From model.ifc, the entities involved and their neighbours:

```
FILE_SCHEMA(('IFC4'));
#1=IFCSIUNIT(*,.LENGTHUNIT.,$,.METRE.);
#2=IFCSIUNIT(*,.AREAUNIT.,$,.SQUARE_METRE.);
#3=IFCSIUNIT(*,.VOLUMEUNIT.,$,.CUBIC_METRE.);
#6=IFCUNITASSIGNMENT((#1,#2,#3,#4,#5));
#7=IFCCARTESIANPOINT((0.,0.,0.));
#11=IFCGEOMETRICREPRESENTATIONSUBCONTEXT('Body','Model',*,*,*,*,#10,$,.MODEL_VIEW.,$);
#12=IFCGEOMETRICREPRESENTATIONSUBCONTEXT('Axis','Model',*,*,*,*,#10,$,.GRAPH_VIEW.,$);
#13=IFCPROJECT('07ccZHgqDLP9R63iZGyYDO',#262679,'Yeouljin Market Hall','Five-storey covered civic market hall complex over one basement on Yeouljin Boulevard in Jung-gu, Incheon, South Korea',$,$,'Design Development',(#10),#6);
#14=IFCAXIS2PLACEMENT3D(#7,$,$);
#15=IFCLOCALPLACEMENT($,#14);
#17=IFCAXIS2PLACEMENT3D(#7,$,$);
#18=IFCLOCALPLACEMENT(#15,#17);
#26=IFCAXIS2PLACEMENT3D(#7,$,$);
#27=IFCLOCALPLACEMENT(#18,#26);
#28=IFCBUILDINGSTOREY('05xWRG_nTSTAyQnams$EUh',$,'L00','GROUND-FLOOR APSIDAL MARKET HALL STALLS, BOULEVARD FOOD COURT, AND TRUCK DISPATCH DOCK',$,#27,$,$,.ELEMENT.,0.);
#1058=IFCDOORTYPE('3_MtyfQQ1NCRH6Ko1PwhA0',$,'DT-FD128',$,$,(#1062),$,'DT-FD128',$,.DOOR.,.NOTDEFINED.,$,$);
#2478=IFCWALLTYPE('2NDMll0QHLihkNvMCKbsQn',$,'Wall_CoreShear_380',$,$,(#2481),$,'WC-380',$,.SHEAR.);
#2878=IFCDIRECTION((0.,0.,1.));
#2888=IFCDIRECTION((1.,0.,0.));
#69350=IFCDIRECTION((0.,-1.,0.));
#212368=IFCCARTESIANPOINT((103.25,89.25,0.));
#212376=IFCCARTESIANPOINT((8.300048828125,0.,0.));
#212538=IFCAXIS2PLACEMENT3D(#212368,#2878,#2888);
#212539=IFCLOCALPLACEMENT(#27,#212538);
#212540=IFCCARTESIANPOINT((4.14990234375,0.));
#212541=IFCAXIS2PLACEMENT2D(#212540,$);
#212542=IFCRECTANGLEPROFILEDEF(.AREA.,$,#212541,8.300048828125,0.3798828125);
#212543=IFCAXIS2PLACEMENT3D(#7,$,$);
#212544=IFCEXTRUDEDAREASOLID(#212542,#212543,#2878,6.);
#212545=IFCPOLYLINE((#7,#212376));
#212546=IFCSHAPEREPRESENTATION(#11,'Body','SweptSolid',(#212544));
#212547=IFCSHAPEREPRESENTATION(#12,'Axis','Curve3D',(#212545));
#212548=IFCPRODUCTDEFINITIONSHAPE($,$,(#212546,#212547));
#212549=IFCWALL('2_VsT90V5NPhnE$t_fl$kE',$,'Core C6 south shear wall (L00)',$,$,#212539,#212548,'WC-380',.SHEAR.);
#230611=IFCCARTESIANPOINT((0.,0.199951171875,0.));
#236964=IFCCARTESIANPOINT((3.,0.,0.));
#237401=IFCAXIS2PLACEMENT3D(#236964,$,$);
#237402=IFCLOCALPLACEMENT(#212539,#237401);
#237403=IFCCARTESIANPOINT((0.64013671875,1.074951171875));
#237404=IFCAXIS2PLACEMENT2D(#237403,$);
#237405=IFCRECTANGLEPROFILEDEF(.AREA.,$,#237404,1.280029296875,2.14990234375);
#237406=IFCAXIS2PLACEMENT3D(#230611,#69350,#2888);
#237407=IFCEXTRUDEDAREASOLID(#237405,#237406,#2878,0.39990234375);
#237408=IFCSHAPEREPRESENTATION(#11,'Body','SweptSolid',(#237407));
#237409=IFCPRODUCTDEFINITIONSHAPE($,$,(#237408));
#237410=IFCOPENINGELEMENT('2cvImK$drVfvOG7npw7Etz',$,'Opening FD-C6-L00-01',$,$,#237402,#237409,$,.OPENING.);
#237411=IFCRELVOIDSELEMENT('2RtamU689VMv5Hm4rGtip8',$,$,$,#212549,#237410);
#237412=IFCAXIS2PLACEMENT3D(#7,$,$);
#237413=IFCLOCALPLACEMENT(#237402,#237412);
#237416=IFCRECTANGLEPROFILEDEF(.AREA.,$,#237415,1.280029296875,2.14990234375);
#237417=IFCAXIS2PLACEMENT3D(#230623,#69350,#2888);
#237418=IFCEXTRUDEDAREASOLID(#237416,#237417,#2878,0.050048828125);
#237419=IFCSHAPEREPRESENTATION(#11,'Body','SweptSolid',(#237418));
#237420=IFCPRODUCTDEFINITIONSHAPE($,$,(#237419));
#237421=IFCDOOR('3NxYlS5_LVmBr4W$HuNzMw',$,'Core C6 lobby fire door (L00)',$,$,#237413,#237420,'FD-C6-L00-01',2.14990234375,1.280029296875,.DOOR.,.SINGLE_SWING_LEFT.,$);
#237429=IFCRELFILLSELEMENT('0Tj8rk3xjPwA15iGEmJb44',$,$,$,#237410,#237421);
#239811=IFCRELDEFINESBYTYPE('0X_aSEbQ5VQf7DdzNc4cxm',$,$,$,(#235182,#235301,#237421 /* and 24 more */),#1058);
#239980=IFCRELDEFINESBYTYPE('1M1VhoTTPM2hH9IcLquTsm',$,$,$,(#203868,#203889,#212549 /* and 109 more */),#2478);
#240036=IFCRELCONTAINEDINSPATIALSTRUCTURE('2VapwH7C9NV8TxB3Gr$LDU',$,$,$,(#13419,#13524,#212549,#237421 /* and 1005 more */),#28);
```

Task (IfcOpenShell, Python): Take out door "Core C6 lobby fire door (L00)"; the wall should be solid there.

```python
import ifcopenshell
import ifcopenshell.api.feature
import ifcopenshell.api.root
import ifcopenshell.geom
import ifcopenshell.util.shape

model = ifcopenshell.open("model.ifc")
settings = ifcopenshell.geom.settings()


def volume(element):
    """Net volume in cubic metres, openings subtracted."""
    shape = ifcopenshell.geom.create_shape(settings, element)
    return ifcopenshell.util.shape.get_volume(shape.geometry)


door = model.by_guid("3NxYlS5_LVmBr4W$HuNzMw")
opening = door.FillsVoids[0].RelatingOpeningElement
wall = opening.VoidsElements[0].RelatingBuildingElement
before = volume(wall)

ifcopenshell.api.root.remove_product(model, product=door)
ifcopenshell.api.feature.remove_feature(model, feature=opening)

after = volume(wall)

print(f"wall volume {before:.3f} -> {after:.3f} m3")

model.write("model_v2.ifc")
```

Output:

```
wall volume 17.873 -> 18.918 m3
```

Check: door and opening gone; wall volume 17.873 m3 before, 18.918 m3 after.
